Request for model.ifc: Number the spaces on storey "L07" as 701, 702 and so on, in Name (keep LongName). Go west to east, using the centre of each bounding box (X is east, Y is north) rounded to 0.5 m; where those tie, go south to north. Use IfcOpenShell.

First a look at what the model holds.

```python
import ifcopenshell
import ifcopenshell.util.element
import ifcopenshell.util.placement

model = ifcopenshell.open("model.ifc")
print(model.schema)
storey = next(s for s in model.by_type("IfcBuildingStorey") if s.Name == "L07")
spaces = [e for e in ifcopenshell.util.element.get_decomposition(storey) if e.is_a("IfcSpace")]
for e in sorted(spaces, key=lambda e: e.id()):
    origin = ifcopenshell.util.placement.get_local_placement(e.ObjectPlacement)[:3, 3]
    print(e.id(), e.Name, e.LongName, origin.round(2) + 0.0, sep=" | ")
```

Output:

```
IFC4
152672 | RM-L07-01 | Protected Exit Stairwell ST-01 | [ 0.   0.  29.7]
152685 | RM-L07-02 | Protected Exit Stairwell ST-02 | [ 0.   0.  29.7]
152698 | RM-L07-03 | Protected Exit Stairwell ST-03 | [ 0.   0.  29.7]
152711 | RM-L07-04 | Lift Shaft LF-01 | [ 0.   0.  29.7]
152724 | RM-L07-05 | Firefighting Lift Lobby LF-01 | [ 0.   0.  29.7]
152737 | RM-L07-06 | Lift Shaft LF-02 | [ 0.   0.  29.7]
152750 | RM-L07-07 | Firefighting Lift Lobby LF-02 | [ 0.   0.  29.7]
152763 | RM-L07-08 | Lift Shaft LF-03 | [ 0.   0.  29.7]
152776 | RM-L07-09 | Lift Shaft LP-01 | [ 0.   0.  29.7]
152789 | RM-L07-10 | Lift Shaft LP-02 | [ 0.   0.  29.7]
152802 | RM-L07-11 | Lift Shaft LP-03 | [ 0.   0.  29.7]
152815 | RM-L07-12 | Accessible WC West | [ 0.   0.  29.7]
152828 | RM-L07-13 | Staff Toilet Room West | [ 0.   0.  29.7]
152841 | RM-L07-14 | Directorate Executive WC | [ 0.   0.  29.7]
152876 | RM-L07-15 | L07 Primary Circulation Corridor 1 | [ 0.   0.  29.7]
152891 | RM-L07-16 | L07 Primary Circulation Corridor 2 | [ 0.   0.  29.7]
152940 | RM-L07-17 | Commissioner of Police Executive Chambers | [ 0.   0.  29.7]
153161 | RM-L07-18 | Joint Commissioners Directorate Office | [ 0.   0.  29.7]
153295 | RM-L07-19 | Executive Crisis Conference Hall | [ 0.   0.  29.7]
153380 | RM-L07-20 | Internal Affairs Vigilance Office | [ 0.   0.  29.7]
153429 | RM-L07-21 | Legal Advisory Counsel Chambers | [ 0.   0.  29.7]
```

```python
import ifcopenshell
import ifcopenshell.geom
import ifcopenshell.util.element
import ifcopenshell.util.shape

model = ifcopenshell.open("model.ifc")
settings = ifcopenshell.geom.settings()
settings.set("use-world-coords", True)


def centre(element):
    shape = ifcopenshell.geom.create_shape(settings, element)
    return ifcopenshell.util.shape.get_bbox_centroid(shape.geometry)


storey = next(s for s in model.by_type("IfcBuildingStorey") if s.Name == "L07")
spaces = [e for e in ifcopenshell.util.element.get_decomposition(storey) if e.is_a("IfcSpace")]

# Insertion points can sit at a corner or the storey origin, so sort by the geometry (in metres).
centres = {e: centre(e) for e in spaces}
spaces.sort(key=lambda e: (round(centres[e][0] / 0.5), centres[e][1]))

for i, e in enumerate(spaces, start=1):
    number = f"7{i:02d}"
    e.Name = number
    print(e.id(), number)

model.write("model_rev.ifc")
```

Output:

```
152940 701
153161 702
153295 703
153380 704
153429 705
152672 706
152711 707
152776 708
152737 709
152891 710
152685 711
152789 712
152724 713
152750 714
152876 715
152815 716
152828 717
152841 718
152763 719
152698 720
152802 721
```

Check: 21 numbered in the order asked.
